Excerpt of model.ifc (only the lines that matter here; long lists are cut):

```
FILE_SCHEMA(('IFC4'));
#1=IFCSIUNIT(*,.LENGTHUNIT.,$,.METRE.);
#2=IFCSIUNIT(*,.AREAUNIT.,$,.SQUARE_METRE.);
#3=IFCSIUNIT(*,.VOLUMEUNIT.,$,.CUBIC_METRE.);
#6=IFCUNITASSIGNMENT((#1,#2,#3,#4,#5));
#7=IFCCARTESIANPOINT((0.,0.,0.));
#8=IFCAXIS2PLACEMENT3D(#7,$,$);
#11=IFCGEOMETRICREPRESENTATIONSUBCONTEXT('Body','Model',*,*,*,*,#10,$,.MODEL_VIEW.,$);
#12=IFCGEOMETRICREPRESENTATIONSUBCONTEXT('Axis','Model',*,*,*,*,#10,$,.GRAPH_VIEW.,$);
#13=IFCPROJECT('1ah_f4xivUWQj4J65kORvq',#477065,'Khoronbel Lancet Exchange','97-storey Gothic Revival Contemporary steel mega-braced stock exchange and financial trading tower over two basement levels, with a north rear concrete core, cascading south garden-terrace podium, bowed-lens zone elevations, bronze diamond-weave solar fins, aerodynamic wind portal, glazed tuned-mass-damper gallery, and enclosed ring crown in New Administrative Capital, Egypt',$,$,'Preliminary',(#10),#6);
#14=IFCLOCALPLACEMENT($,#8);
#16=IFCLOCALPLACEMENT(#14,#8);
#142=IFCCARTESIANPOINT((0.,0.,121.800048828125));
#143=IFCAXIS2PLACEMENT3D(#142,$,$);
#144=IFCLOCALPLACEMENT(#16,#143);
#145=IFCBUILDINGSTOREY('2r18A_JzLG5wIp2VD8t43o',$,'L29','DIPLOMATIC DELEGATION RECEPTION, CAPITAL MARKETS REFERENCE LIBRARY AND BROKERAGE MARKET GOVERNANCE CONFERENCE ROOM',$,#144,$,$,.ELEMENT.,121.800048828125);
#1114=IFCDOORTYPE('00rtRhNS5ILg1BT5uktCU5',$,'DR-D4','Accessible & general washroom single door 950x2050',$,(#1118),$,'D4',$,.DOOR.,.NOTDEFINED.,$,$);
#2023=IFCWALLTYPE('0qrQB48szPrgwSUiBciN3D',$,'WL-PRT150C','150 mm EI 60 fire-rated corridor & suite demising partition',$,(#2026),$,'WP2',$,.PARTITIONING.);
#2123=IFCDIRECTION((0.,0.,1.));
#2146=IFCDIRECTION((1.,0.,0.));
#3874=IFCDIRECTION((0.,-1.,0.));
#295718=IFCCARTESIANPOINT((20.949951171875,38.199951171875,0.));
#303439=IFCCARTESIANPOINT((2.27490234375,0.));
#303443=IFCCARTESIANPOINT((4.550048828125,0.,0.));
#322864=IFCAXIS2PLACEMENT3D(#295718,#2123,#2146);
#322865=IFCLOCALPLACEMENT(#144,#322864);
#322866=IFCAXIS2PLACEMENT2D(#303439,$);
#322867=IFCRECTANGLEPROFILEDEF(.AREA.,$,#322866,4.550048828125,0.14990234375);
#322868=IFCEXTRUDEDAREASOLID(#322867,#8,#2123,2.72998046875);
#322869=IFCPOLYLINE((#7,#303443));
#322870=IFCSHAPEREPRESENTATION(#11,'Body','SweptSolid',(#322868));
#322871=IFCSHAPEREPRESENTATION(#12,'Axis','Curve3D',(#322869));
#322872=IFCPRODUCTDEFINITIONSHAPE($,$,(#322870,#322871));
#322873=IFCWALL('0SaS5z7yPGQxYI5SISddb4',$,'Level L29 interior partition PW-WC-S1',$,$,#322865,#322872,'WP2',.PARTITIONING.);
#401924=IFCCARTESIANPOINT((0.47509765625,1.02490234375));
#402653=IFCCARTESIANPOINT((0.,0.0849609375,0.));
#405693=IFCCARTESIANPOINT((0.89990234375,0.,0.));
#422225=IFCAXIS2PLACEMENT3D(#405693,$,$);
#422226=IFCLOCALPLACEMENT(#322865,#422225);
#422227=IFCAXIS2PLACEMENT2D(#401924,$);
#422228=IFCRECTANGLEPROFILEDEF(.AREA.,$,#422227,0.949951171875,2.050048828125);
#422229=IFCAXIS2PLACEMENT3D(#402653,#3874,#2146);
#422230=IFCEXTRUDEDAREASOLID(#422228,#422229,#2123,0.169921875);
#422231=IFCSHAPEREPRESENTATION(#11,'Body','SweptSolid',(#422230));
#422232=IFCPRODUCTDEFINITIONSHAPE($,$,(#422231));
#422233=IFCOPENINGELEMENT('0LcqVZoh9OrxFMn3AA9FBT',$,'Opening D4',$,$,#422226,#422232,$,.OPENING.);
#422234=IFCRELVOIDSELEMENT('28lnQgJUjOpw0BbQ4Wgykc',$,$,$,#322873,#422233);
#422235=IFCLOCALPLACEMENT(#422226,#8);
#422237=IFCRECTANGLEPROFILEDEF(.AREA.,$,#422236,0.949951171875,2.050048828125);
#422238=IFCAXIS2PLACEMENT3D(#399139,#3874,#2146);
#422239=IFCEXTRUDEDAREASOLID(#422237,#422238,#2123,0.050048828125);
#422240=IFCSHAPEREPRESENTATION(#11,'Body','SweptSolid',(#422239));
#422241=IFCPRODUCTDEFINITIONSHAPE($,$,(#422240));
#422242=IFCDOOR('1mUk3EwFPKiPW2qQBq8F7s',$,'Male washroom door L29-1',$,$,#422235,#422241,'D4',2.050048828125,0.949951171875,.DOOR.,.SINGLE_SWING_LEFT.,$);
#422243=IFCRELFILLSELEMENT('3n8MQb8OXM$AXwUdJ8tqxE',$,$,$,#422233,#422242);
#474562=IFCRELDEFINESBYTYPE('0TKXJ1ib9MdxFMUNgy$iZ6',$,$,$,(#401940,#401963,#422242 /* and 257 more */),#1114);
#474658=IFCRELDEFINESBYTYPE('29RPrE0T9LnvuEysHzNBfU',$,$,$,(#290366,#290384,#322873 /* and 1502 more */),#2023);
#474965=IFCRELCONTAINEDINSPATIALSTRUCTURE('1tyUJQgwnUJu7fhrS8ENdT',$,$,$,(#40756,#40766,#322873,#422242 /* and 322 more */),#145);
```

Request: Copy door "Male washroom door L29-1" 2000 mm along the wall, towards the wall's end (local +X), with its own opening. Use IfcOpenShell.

```python
import ifcopenshell
import ifcopenshell.api.feature
import ifcopenshell.api.geometry
import ifcopenshell.api.root
import ifcopenshell.geom
import ifcopenshell.util.element
import ifcopenshell.util.placement
import ifcopenshell.util.shape
import ifcopenshell.util.unit

model = ifcopenshell.open("model.ifc")
unit_scale = ifcopenshell.util.unit.calculate_unit_scale(model)
settings = ifcopenshell.geom.settings()


def volume(element):
    """Net volume in cubic metres, openings subtracted."""
    shape = ifcopenshell.geom.create_shape(settings, element)
    return ifcopenshell.util.shape.get_volume(shape.geometry)


door = model.by_guid("1mUk3EwFPKiPW2qQBq8F7s")
opening = door.FillsVoids[0].RelatingOpeningElement
wall = opening.VoidsElements[0].RelatingBuildingElement
before = volume(wall)
shift = ifcopenshell.util.placement.get_local_placement(wall.ObjectPlacement)[:3, 0] * 2 / unit_scale

# copy_class copies the void relationship, type, container and properties, but no geometry.
new_opening = ifcopenshell.api.root.copy_class(model, product=opening)
new_opening.Representation = ifcopenshell.util.element.copy_deep(
    model, opening.Representation, exclude=["IfcGeometricRepresentationContext", "IfcRepresentationMap"]
)
new_door = ifcopenshell.api.root.copy_class(model, product=door)
new_door.Representation = ifcopenshell.util.element.copy_deep(
    model, door.Representation, exclude=["IfcGeometricRepresentationContext", "IfcRepresentationMap"]
)
new_door.Tag = None
ifcopenshell.api.feature.add_filling(model, opening=new_opening, element=new_door)

for old, new in ((opening, new_opening), (door, new_door)):
    matrix = ifcopenshell.util.placement.get_local_placement(old.ObjectPlacement)
    matrix[:3, 3] += shift
    ifcopenshell.api.geometry.edit_object_placement(model, product=new, matrix=matrix, is_si=False)

after = volume(wall)

print(f"wall volume {before:.3f} -> {after:.3f} m3")

model.write("model_edited.ifc")
```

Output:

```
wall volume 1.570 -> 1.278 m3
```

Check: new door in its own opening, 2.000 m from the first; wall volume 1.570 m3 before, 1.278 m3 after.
